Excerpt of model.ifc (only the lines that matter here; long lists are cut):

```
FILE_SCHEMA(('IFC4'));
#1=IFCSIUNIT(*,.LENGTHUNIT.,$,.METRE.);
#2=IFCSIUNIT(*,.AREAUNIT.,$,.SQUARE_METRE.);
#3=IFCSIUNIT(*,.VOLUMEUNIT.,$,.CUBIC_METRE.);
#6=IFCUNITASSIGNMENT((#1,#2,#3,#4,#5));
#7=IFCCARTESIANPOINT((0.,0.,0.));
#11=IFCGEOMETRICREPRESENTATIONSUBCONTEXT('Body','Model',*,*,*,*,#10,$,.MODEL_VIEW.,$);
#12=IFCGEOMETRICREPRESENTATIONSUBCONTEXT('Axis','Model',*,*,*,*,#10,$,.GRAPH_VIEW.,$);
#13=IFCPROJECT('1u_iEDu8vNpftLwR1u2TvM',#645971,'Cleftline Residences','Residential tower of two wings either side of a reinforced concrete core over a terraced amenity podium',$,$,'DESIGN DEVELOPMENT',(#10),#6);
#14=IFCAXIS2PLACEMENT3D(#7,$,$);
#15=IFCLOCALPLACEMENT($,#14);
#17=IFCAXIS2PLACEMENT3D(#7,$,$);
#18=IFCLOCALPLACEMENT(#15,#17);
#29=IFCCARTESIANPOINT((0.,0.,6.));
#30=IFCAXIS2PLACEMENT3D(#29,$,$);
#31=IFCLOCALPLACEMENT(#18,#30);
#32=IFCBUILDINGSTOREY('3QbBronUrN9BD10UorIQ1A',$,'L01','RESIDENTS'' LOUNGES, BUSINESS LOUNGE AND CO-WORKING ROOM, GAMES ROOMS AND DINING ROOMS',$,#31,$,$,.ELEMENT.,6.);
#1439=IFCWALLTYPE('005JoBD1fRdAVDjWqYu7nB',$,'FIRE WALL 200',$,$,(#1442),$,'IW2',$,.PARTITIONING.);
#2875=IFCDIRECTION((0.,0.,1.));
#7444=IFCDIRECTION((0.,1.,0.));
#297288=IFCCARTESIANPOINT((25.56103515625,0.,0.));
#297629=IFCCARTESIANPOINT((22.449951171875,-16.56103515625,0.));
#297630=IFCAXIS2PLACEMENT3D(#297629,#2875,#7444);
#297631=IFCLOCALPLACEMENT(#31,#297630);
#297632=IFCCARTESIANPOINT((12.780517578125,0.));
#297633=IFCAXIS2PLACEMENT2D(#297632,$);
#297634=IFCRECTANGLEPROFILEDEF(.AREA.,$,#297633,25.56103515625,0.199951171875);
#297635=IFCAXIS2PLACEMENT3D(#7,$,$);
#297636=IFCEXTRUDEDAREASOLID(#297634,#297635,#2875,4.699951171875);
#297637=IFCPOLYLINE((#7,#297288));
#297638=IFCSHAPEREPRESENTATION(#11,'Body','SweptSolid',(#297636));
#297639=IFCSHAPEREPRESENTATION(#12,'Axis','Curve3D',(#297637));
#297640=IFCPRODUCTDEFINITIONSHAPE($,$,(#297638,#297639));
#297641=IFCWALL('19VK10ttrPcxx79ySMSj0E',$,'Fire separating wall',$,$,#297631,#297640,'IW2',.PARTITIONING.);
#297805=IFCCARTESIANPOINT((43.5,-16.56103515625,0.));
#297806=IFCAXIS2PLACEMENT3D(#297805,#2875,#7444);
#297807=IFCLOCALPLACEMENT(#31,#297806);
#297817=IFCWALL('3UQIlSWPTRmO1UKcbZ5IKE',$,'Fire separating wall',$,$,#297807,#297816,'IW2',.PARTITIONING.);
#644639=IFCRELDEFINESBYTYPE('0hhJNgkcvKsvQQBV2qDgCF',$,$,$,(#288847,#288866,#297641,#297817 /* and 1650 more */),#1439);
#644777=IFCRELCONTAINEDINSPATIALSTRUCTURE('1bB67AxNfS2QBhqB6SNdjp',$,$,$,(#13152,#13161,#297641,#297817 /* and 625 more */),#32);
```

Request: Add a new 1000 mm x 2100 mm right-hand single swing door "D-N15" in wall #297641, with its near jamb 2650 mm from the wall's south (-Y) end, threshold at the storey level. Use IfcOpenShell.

```python
import numpy as np
import ifcopenshell
import ifcopenshell.api.feature
import ifcopenshell.api.geometry
import ifcopenshell.api.root
import ifcopenshell.api.spatial
import ifcopenshell.geom
import ifcopenshell.util.element
import ifcopenshell.util.placement
import ifcopenshell.util.representation
import ifcopenshell.util.shape
import ifcopenshell.util.unit

model = ifcopenshell.open("model.ifc")
unit_scale = ifcopenshell.util.unit.calculate_unit_scale(model)
settings = ifcopenshell.geom.settings()


def volume(element):
    """Net volume in cubic metres, openings subtracted."""
    shape = ifcopenshell.geom.create_shape(settings, element)
    return ifcopenshell.util.shape.get_volume(shape.geometry)


wall = model.by_guid("19VK10ttrPcxx79ySMSj0E")
storey = ifcopenshell.util.element.get_container(wall, ifc_class="IfcBuildingStorey")
context = ifcopenshell.util.representation.get_context(model, "Model", "Body", "MODEL_VIEW")
before = volume(wall)

width, height, from_end, sill = 1, 2.1, 2.65, 0.0  # metres

# The wall runs along its own X axis, and the end named is its -X end.
wall_shape = ifcopenshell.geom.create_shape(settings, wall)
x, y, z = ifcopenshell.util.shape.get_vertices(wall_shape.geometry).T
start = x.min() + from_end
face, thickness = float(y.min()), float(y.max() - y.min())
wall_matrix = ifcopenshell.util.placement.get_local_placement(wall.ObjectPlacement)
level = ifcopenshell.util.placement.get_local_placement(storey.ObjectPlacement)[2, 3]


def in_wall(x, y):
    """Placement at x, y metres in the wall's axes, at sill height."""
    matrix = wall_matrix.copy()
    matrix[:, 3] = wall_matrix @ np.array([x / unit_scale, y / unit_scale, 0.0, 1.0])
    matrix[2, 3] = level + sill / unit_scale
    return matrix


# Opening: a box that overshoots both wall faces by 50 mm.
opening = ifcopenshell.api.root.create_entity(model, ifc_class="IfcOpeningElement", predefined_type="OPENING")
box = ifcopenshell.api.geometry.add_wall_representation(
    model, context=context, length=width, height=height, thickness=thickness + 0.1
)
ifcopenshell.api.geometry.assign_representation(model, product=opening, representation=box)
ifcopenshell.api.geometry.edit_object_placement(model, product=opening, matrix=in_wall(start, face - 0.05), is_si=False)
ifcopenshell.api.feature.add_feature(model, feature=opening, element=wall)

door = ifcopenshell.api.root.create_entity(model, ifc_class="IfcDoor", name="D-N15", predefined_type="DOOR")
door.OverallWidth, door.OverallHeight = width / unit_scale, height / unit_scale
door.OperationType = "SINGLE_SWING_RIGHT"
body = ifcopenshell.api.geometry.add_door_representation(
    model,
    context=context,
    overall_width=door.OverallWidth,
    overall_height=door.OverallHeight,
    operation_type="SINGLE_SWING_RIGHT",
    lining_properties={"LiningDepth": thickness / unit_scale, "ThresholdDepth": thickness / unit_scale},
)
ifcopenshell.api.geometry.assign_representation(model, product=door, representation=body)
ifcopenshell.api.spatial.assign_container(model, products=[door], relating_structure=storey)
ifcopenshell.api.feature.add_filling(model, opening=opening, element=door)

# The lining spans the wall, so the door starts at the wall face.
ifcopenshell.api.geometry.edit_object_placement(model, product=door, matrix=in_wall(start, face), is_si=False)

after = volume(wall)

print(f"wall volume {before:.3f} -> {after:.3f} m3")

model.write("model_v2.ifc")
```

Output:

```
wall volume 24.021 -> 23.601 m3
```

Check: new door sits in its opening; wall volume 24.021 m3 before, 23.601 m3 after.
